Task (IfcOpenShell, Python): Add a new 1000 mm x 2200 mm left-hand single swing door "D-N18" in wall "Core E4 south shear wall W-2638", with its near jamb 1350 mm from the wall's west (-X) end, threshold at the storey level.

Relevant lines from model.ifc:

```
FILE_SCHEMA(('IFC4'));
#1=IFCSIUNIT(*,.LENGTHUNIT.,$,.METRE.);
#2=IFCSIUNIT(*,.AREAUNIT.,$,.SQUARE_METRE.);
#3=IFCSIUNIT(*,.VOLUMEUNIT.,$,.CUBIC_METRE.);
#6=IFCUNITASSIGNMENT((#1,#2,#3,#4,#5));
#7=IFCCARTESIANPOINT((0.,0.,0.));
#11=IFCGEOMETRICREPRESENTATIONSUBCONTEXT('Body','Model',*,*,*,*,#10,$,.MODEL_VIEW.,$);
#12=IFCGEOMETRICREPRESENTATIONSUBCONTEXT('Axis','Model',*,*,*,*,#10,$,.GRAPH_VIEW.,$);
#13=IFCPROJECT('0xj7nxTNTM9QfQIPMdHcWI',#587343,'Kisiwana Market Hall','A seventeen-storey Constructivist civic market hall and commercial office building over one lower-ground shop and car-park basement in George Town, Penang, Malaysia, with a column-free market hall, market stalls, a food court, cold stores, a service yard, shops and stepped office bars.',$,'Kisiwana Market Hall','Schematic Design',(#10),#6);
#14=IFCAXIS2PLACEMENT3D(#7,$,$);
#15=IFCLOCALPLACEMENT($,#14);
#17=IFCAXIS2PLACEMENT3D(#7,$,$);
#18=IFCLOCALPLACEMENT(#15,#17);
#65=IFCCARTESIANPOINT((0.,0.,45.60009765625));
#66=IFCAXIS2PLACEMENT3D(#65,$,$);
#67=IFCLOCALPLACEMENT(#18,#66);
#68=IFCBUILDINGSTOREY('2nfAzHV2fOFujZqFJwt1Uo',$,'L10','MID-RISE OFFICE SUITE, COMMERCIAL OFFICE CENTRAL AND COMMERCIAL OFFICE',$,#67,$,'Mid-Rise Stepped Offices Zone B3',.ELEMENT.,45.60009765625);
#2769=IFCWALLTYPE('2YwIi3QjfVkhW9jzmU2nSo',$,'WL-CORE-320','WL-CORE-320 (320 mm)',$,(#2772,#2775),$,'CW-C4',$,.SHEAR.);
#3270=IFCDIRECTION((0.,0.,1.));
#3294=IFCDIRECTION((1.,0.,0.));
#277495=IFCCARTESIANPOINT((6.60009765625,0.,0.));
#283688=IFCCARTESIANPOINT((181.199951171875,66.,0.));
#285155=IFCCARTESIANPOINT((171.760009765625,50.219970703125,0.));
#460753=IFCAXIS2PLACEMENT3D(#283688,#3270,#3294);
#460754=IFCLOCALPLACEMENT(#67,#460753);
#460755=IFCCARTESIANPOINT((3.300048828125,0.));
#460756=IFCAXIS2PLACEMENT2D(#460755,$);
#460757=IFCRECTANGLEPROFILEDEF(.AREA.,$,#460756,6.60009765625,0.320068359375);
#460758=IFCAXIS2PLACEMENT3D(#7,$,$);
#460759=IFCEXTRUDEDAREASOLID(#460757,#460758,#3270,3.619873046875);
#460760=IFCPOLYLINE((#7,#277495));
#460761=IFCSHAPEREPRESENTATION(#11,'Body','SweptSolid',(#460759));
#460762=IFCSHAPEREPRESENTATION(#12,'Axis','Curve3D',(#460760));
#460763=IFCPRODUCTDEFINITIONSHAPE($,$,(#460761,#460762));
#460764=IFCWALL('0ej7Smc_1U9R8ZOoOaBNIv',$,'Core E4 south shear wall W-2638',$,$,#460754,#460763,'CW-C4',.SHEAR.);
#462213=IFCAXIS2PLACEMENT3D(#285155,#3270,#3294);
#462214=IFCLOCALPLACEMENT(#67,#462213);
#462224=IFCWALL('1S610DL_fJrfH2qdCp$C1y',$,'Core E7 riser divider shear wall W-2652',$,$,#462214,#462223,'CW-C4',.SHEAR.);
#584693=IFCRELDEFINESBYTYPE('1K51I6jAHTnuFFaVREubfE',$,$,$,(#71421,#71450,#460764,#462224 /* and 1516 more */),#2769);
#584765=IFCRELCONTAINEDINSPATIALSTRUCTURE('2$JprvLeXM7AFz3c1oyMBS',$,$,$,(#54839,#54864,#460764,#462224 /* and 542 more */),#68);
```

```python
import numpy as np
import ifcopenshell
import ifcopenshell.api.feature
import ifcopenshell.api.geometry
import ifcopenshell.api.root
import ifcopenshell.api.spatial
import ifcopenshell.geom
import ifcopenshell.util.element
import ifcopenshell.util.placement
import ifcopenshell.util.representation
import ifcopenshell.util.shape
import ifcopenshell.util.unit

model = ifcopenshell.open("model.ifc")
unit_scale = ifcopenshell.util.unit.calculate_unit_scale(model)
settings = ifcopenshell.geom.settings()


def volume(element):
    """Net volume in cubic metres, openings subtracted."""
    shape = ifcopenshell.geom.create_shape(settings, element)
    return ifcopenshell.util.shape.get_volume(shape.geometry)


wall = model.by_id(460764)
storey = ifcopenshell.util.element.get_container(wall, ifc_class="IfcBuildingStorey")
context = ifcopenshell.util.representation.get_context(model, "Model", "Body", "MODEL_VIEW")
before = volume(wall)

width, height, from_end, sill = 1, 2.2, 1.35, 0.0  # metres

# The wall runs along its own X axis, and the end named is its -X end.
wall_shape = ifcopenshell.geom.create_shape(settings, wall)
x, y, z = ifcopenshell.util.shape.get_vertices(wall_shape.geometry).T
start = x.min() + from_end
face, thickness = float(y.min()), float(y.max() - y.min())
wall_matrix = ifcopenshell.util.placement.get_local_placement(wall.ObjectPlacement)
level = ifcopenshell.util.placement.get_local_placement(storey.ObjectPlacement)[2, 3]


def in_wall(x, y):
    """Placement at x, y metres in the wall's axes, at sill height."""
    matrix = wall_matrix.copy()
    matrix[:, 3] = wall_matrix @ np.array([x / unit_scale, y / unit_scale, 0.0, 1.0])
    matrix[2, 3] = level + sill / unit_scale
    return matrix


# Opening: a box that overshoots both wall faces by 50 mm.
opening = ifcopenshell.api.root.create_entity(model, ifc_class="IfcOpeningElement", predefined_type="OPENING")
box = ifcopenshell.api.geometry.add_wall_representation(
    model, context=context, length=width, height=height, thickness=thickness + 0.1
)
ifcopenshell.api.geometry.assign_representation(model, product=opening, representation=box)
ifcopenshell.api.geometry.edit_object_placement(model, product=opening, matrix=in_wall(start, face - 0.05), is_si=False)
ifcopenshell.api.feature.add_feature(model, feature=opening, element=wall)

door = ifcopenshell.api.root.create_entity(model, ifc_class="IfcDoor", name="D-N18", predefined_type="DOOR")
door.OverallWidth, door.OverallHeight = width / unit_scale, height / unit_scale
door.OperationType = "SINGLE_SWING_LEFT"
body = ifcopenshell.api.geometry.add_door_representation(
    model,
    context=context,
    overall_width=door.OverallWidth,
    overall_height=door.OverallHeight,
    operation_type="SINGLE_SWING_LEFT",
    lining_properties={"LiningDepth": thickness / unit_scale, "ThresholdDepth": thickness / unit_scale},
)
ifcopenshell.api.geometry.assign_representation(model, product=door, representation=body)
ifcopenshell.api.spatial.assign_container(model, products=[door], relating_structure=storey)
ifcopenshell.api.feature.add_filling(model, opening=opening, element=door)

# The lining spans the wall, so the door starts at the wall face.
ifcopenshell.api.geometry.edit_object_placement(model, product=door, matrix=in_wall(start, face), is_si=False)

after = volume(wall)

print(f"wall volume {before:.3f} -> {after:.3f} m3")

model.write("model_rev.ifc")
```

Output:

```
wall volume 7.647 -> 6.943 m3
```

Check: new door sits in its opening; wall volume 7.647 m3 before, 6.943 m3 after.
